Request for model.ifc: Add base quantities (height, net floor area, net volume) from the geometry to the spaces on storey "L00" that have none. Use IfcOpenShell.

First a look at what the model holds.

```python
import ifcopenshell
import ifcopenshell.util.element
import ifcopenshell.util.unit

model = ifcopenshell.open("model.ifc")
print(model.schema)
for unit_type in ("LENGTHUNIT", "AREAUNIT", "VOLUMEUNIT"):
    print(unit_type, ifcopenshell.util.unit.calculate_unit_scale(model, unit_type))
storey = next(s for s in model.by_type("IfcBuildingStorey") if s.Name == "L00")
spaces = [e for e in ifcopenshell.util.element.get_decomposition(storey) if e.is_a("IfcSpace")]
for e in sorted(spaces, key=lambda e: e.id()):
    print(e.id(), e.is_a(), e.Name, list(ifcopenshell.util.element.get_psets(e, qtos_only=True)), sep=" | ")
```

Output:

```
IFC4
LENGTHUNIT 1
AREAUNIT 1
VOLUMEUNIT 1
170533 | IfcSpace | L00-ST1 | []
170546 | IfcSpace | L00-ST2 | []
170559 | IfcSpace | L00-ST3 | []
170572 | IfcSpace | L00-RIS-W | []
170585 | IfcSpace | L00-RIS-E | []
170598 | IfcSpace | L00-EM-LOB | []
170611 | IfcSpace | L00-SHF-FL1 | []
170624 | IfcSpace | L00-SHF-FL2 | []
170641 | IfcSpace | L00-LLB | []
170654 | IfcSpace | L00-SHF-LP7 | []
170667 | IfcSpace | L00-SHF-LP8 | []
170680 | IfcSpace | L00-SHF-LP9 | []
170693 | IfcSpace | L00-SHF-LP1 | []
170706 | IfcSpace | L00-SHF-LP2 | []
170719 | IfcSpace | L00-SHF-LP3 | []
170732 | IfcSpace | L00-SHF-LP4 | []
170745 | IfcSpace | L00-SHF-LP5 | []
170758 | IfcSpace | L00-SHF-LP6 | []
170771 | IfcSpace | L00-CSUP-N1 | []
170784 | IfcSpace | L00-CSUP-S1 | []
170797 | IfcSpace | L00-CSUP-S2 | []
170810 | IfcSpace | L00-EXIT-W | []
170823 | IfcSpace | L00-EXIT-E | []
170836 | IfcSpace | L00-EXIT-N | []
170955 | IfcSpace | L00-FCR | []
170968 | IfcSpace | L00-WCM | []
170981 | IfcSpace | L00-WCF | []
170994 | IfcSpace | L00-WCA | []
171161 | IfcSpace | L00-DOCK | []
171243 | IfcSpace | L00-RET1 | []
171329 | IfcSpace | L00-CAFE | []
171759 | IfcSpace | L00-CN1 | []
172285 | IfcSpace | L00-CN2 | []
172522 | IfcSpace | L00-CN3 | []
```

```python
import ifcopenshell
import ifcopenshell.api.pset
import ifcopenshell.geom
import ifcopenshell.util.element
import ifcopenshell.util.shape
import ifcopenshell.util.unit

model = ifcopenshell.open("model.ifc")
unit_scale = ifcopenshell.util.unit.calculate_unit_scale(model)
area_scale = ifcopenshell.util.unit.calculate_unit_scale(model, "AREAUNIT")
volume_scale = ifcopenshell.util.unit.calculate_unit_scale(model, "VOLUMEUNIT")
settings = ifcopenshell.geom.settings()

storey = next(s for s in model.by_type("IfcBuildingStorey") if s.Name == "L00")
spaces = [e for e in ifcopenshell.util.element.get_decomposition(storey) if e.is_a("IfcSpace")]

for e in sorted(spaces, key=lambda e: e.id()):
    if ifcopenshell.util.element.get_psets(e, qtos_only=True, should_inherit=False):
        continue
    # Geometry comes back in metres, in the element's own axes.
    shape = ifcopenshell.geom.create_shape(settings, e)
    values = {
        "Height": ifcopenshell.util.shape.get_z(shape.geometry) / unit_scale,
        "NetFloorArea": ifcopenshell.util.shape.get_footprint_area(shape.geometry) / area_scale,
        "NetVolume": ifcopenshell.util.shape.get_volume(shape.geometry) / volume_scale,
    }
    qto = ifcopenshell.api.pset.add_qto(model, product=e, name="Qto_SpaceBaseQuantities")
    ifcopenshell.api.pset.edit_qto(model, qto=qto, properties=values)
    print(e.id(), {k: round(v, 3) for k, v in values.items()})

model.write("model-out.ifc")
```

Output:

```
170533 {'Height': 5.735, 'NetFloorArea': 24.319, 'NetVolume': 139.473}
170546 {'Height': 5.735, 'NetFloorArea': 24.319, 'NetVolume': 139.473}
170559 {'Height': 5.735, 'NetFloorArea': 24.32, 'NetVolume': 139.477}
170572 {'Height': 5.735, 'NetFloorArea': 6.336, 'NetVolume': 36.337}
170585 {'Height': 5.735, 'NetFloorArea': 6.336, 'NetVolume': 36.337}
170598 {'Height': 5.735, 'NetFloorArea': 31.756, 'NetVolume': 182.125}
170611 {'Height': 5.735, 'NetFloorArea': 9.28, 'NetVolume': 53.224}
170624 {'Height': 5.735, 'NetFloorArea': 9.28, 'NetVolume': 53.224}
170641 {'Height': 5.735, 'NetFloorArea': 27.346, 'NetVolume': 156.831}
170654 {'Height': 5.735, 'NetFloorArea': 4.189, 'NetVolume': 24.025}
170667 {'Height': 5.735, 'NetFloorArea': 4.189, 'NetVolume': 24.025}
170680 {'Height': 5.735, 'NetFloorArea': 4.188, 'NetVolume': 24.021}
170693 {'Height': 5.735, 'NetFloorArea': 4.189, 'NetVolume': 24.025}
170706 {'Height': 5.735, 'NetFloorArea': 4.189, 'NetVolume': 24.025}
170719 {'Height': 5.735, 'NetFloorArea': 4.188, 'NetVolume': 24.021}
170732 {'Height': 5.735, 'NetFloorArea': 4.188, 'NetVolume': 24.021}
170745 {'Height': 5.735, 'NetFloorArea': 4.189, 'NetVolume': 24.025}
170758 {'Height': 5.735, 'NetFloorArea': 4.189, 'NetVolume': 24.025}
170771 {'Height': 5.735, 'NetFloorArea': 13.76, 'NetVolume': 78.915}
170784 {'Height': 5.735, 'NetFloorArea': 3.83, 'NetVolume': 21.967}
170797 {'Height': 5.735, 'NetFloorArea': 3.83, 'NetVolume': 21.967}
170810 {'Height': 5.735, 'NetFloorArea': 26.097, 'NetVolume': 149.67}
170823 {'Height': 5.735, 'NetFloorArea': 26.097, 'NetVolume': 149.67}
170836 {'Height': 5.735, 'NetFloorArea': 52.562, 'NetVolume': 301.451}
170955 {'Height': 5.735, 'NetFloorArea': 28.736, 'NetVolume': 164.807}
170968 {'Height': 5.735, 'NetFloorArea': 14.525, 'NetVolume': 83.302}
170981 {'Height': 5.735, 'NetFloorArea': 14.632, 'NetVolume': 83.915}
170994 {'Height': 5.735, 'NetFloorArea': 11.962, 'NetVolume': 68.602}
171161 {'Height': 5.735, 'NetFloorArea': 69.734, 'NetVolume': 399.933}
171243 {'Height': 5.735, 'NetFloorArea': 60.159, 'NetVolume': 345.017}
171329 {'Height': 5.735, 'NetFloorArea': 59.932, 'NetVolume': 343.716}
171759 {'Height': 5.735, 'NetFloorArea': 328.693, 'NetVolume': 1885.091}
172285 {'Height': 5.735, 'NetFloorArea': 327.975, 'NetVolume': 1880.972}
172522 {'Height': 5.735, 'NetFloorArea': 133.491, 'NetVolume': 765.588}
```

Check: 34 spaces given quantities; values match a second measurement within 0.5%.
